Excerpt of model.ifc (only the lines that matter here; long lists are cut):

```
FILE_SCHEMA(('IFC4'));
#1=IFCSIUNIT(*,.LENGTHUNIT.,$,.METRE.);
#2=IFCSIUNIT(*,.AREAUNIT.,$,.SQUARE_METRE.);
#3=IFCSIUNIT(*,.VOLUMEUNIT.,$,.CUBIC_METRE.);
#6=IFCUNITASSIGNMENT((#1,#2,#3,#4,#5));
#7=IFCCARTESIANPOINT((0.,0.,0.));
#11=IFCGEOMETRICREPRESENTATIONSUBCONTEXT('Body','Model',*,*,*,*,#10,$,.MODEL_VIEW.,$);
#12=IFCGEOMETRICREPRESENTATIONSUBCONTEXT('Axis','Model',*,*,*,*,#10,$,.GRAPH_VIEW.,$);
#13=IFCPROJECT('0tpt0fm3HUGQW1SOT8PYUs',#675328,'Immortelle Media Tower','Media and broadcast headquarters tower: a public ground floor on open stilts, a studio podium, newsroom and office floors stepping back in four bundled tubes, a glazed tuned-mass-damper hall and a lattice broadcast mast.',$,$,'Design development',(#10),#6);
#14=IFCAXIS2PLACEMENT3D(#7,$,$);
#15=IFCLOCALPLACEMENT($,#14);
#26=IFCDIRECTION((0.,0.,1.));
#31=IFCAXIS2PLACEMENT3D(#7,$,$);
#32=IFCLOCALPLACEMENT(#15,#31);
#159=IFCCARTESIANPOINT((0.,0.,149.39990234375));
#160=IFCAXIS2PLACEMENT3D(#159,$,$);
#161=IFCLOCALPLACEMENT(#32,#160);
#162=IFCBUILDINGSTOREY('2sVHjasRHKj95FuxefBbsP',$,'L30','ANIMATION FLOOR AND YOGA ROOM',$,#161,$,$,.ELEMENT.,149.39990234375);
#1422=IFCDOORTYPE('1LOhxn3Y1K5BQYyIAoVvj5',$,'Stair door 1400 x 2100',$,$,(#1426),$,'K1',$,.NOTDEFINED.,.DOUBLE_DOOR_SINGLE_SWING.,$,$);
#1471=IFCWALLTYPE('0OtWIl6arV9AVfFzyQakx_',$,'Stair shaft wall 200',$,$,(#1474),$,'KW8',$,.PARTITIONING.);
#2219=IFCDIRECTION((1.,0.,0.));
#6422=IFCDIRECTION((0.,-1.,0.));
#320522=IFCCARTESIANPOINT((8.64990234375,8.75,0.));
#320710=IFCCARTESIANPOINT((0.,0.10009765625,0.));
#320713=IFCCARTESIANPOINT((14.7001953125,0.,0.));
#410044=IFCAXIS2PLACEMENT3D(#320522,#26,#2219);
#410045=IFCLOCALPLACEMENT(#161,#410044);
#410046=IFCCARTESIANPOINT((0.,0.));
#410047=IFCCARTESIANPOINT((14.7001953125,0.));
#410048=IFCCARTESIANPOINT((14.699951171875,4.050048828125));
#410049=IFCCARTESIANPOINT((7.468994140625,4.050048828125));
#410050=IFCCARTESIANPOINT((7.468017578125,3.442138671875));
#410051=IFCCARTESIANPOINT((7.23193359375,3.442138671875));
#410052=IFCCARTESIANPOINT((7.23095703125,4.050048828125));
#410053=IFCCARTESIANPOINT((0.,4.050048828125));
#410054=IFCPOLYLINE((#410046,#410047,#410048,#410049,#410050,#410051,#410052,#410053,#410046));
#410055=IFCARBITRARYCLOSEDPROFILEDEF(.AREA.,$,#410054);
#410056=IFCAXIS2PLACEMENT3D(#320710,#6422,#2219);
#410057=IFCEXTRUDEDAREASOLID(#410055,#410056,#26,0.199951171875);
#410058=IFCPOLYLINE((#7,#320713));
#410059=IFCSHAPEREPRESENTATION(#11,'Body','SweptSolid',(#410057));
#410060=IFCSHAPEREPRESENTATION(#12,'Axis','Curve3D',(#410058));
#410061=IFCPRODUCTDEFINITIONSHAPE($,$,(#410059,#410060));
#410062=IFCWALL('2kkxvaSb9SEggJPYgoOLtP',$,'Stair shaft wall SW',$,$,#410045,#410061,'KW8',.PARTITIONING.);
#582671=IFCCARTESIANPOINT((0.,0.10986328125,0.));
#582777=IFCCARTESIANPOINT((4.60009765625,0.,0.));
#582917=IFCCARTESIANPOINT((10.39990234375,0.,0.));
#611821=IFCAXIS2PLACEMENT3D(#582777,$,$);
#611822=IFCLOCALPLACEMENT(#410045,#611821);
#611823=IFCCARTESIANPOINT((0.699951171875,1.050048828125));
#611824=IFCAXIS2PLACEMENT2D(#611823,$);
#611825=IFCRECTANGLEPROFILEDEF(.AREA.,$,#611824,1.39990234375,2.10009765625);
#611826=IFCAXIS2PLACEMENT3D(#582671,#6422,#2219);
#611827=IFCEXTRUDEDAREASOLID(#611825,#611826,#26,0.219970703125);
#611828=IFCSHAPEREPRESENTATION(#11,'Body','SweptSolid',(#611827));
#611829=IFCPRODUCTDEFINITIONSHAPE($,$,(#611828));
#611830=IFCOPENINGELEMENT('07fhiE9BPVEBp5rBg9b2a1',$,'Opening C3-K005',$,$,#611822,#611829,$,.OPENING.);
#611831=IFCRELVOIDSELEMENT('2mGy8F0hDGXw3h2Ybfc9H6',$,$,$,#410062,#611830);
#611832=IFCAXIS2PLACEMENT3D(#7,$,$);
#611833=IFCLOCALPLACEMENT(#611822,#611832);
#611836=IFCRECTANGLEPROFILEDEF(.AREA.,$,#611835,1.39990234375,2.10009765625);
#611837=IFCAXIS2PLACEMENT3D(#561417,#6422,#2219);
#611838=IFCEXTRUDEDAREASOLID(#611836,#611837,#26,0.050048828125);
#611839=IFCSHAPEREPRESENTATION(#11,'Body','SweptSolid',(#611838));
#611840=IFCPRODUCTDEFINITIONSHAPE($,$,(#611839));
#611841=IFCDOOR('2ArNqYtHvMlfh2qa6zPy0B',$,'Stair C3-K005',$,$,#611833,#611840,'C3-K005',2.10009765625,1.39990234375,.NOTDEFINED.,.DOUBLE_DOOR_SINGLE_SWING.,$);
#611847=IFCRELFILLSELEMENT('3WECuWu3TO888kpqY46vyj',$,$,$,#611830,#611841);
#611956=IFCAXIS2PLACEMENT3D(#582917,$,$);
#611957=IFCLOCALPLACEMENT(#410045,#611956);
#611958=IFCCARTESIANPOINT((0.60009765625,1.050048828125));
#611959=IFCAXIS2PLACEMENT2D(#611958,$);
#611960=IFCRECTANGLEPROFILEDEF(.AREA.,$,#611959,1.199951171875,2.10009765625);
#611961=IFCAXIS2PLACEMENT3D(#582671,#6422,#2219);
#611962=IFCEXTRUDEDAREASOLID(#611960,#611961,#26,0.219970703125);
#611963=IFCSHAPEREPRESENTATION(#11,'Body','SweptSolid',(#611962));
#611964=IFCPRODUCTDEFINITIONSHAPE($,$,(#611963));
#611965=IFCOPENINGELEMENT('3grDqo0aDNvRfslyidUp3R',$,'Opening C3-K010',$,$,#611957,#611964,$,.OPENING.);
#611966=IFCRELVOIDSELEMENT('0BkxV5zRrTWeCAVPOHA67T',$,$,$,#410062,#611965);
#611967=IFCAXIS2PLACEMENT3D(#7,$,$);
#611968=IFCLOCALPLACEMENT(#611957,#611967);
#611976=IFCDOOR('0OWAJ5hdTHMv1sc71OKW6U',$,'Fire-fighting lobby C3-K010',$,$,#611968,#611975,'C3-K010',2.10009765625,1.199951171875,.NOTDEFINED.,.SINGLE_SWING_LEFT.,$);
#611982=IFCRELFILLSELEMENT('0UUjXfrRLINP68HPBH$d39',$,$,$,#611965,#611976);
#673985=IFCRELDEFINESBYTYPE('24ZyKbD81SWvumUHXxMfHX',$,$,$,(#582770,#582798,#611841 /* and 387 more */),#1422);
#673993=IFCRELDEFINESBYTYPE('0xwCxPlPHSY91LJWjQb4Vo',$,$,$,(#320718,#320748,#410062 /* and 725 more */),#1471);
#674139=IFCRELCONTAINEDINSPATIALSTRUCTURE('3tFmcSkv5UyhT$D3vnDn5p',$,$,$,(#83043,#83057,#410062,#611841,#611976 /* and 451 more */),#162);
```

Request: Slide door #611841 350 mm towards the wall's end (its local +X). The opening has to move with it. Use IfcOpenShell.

```python
import ifcopenshell
import ifcopenshell.api.geometry
import ifcopenshell.util.placement
import ifcopenshell.util.unit

model = ifcopenshell.open("model.ifc")
unit_scale = ifcopenshell.util.unit.calculate_unit_scale(model)

door = model.by_guid("2ArNqYtHvMlfh2qa6zPy0B")
opening = door.FillsVoids[0].RelatingOpeningElement
wall = opening.VoidsElements[0].RelatingBuildingElement

wall_matrix = ifcopenshell.util.placement.get_local_placement(wall.ObjectPlacement)
shift = wall_matrix[:3, 0] * 0.35 / unit_scale
before = ifcopenshell.util.placement.get_local_placement(door.ObjectPlacement)[:3, 3].copy()

# The door is placed relative to its opening, so it follows when the opening moves.
matrix = ifcopenshell.util.placement.get_local_placement(opening.ObjectPlacement)
matrix[:3, 3] += shift
ifcopenshell.api.geometry.edit_object_placement(
    model, product=opening, matrix=matrix, is_si=False, should_transform_children=True
)

after = ifcopenshell.util.placement.get_local_placement(door.ObjectPlacement)[:3, 3]
print("door moved by", (after - before).round(3) + 0.0)

model.write("model_updated.ifc")
```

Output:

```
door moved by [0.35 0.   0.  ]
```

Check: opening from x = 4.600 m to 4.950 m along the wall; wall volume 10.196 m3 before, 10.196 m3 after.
